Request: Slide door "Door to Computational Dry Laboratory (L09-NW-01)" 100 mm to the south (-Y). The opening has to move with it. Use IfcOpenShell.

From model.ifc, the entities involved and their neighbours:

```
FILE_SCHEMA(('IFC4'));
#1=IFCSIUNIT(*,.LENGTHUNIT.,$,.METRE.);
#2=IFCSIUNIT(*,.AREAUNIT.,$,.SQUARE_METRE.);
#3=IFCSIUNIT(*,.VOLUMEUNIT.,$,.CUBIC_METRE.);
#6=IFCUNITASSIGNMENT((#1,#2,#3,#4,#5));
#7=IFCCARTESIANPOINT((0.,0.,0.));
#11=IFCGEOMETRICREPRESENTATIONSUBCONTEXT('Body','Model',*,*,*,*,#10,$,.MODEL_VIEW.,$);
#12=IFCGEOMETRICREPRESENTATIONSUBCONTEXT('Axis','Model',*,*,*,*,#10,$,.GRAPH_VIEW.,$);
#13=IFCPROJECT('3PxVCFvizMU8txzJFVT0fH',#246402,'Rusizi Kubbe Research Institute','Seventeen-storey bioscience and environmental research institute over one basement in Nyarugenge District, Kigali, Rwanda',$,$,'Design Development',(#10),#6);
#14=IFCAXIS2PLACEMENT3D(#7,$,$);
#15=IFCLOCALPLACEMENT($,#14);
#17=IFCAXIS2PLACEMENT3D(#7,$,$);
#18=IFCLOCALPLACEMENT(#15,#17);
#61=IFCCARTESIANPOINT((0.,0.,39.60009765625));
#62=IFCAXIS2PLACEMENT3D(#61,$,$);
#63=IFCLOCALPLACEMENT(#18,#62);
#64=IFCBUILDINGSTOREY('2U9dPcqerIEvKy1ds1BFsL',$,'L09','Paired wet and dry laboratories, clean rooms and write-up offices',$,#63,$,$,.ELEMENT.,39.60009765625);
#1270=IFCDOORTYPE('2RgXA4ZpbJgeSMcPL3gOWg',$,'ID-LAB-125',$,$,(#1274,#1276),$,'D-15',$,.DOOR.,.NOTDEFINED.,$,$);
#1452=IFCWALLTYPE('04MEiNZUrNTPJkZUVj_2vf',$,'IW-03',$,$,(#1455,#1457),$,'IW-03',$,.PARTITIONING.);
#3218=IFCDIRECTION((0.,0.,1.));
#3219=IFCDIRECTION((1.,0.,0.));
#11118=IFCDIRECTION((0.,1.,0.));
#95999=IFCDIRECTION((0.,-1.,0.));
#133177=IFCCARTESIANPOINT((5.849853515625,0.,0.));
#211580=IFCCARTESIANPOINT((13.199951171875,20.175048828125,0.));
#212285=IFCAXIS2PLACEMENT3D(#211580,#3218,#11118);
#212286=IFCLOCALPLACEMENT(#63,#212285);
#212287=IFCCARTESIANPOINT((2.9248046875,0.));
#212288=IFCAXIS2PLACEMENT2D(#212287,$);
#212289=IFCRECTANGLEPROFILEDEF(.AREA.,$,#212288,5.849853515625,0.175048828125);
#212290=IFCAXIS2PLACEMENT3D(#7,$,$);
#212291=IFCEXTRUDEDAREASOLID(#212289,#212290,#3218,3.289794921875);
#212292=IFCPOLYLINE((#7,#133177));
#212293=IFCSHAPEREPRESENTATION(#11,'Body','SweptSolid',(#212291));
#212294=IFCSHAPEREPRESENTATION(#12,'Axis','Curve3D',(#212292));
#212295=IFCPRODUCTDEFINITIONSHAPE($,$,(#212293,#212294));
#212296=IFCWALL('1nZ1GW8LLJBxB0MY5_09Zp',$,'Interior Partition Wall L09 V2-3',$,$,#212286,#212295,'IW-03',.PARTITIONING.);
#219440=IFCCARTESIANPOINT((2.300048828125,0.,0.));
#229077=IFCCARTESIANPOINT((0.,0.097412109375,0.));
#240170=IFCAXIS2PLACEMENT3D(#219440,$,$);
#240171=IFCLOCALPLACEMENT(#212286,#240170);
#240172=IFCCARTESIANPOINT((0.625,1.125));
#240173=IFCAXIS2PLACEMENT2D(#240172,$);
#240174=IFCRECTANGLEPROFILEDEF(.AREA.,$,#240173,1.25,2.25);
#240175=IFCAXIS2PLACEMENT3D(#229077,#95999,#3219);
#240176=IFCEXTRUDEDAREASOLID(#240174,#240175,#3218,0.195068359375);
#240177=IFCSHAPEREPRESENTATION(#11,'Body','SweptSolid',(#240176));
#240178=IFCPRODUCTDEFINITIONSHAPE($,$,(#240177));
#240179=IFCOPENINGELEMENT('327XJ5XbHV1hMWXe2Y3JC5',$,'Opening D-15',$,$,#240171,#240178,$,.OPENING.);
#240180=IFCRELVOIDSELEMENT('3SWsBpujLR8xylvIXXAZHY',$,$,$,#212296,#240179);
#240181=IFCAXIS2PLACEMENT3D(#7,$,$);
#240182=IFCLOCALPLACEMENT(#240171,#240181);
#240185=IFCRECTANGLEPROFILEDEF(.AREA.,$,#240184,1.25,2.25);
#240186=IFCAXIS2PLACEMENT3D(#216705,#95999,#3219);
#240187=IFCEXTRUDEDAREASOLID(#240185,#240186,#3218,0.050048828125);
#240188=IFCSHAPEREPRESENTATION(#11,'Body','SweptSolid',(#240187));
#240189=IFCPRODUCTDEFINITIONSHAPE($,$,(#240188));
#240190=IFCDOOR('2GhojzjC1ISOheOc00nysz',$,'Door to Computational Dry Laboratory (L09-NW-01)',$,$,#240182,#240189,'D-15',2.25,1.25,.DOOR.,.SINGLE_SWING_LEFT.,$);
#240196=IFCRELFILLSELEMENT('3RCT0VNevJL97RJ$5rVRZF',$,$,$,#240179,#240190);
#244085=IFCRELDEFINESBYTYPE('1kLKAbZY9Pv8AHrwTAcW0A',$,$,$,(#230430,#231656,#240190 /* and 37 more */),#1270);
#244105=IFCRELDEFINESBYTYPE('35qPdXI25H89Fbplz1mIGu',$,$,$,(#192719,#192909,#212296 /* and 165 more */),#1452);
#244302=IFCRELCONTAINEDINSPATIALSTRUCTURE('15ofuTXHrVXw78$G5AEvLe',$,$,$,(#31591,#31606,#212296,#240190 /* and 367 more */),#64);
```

```python
import ifcopenshell
import ifcopenshell.api.geometry
import ifcopenshell.util.placement
import ifcopenshell.util.unit

model = ifcopenshell.open("model.ifc")
unit_scale = ifcopenshell.util.unit.calculate_unit_scale(model)

door = model.by_guid("2GhojzjC1ISOheOc00nysz")
opening = door.FillsVoids[0].RelatingOpeningElement
wall = opening.VoidsElements[0].RelatingBuildingElement

wall_matrix = ifcopenshell.util.placement.get_local_placement(wall.ObjectPlacement)
shift = wall_matrix[:3, 0] * -0.1 / unit_scale
before = ifcopenshell.util.placement.get_local_placement(door.ObjectPlacement)[:3, 3].copy()

# The door is placed relative to its opening, so it follows when the opening moves.
matrix = ifcopenshell.util.placement.get_local_placement(opening.ObjectPlacement)
matrix[:3, 3] += shift
ifcopenshell.api.geometry.edit_object_placement(
    model, product=opening, matrix=matrix, is_si=False, should_transform_children=True
)

after = ifcopenshell.util.placement.get_local_placement(door.ObjectPlacement)[:3, 3]
print("door moved by", (after - before).round(3) + 0.0)

model.write("model_updated.ifc")
```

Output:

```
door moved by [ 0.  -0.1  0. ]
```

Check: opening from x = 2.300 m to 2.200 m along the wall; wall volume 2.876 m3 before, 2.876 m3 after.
